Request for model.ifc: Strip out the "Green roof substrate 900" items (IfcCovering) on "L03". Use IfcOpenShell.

First a look at what the model holds.

```python
import ifcopenshell
import ifcopenshell.util.element

model = ifcopenshell.open("model.ifc")
print(model.schema)
storey = next(s for s in model.by_type("IfcBuildingStorey") if s.Name == "L03")
coverings = [e for e in ifcopenshell.util.element.get_decomposition(storey) if e.is_a("IfcCovering")]
seen = {}
for e in coverings:
    element_type = ifcopenshell.util.element.get_type(e)
    name = element_type.Name if element_type not in (None, e) else None
    seen[name] = seen.get(name, 0) + 1
for name, count in sorted(seen.items(), key=str):
    print(count, "x", name)
```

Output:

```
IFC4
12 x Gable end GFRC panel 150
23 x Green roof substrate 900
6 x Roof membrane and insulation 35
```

```python
import ifcopenshell
import ifcopenshell.api.root
import ifcopenshell.util.element

model = ifcopenshell.open("model.ifc")

storey = next(s for s in model.by_type("IfcBuildingStorey") if s.Name == "L03")
coverings = [e for e in ifcopenshell.util.element.get_decomposition(storey) if e.is_a("IfcCovering")]
targets = [e for e in coverings if (t := ifcopenshell.util.element.get_type(e)) not in (None, e) and t.Name == "Green roof substrate 900"]

for e in targets:
    ifcopenshell.api.root.remove_product(model, product=e)
print(len(targets), "removed")

model.write("model_v2.ifc")
```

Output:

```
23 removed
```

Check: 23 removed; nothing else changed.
